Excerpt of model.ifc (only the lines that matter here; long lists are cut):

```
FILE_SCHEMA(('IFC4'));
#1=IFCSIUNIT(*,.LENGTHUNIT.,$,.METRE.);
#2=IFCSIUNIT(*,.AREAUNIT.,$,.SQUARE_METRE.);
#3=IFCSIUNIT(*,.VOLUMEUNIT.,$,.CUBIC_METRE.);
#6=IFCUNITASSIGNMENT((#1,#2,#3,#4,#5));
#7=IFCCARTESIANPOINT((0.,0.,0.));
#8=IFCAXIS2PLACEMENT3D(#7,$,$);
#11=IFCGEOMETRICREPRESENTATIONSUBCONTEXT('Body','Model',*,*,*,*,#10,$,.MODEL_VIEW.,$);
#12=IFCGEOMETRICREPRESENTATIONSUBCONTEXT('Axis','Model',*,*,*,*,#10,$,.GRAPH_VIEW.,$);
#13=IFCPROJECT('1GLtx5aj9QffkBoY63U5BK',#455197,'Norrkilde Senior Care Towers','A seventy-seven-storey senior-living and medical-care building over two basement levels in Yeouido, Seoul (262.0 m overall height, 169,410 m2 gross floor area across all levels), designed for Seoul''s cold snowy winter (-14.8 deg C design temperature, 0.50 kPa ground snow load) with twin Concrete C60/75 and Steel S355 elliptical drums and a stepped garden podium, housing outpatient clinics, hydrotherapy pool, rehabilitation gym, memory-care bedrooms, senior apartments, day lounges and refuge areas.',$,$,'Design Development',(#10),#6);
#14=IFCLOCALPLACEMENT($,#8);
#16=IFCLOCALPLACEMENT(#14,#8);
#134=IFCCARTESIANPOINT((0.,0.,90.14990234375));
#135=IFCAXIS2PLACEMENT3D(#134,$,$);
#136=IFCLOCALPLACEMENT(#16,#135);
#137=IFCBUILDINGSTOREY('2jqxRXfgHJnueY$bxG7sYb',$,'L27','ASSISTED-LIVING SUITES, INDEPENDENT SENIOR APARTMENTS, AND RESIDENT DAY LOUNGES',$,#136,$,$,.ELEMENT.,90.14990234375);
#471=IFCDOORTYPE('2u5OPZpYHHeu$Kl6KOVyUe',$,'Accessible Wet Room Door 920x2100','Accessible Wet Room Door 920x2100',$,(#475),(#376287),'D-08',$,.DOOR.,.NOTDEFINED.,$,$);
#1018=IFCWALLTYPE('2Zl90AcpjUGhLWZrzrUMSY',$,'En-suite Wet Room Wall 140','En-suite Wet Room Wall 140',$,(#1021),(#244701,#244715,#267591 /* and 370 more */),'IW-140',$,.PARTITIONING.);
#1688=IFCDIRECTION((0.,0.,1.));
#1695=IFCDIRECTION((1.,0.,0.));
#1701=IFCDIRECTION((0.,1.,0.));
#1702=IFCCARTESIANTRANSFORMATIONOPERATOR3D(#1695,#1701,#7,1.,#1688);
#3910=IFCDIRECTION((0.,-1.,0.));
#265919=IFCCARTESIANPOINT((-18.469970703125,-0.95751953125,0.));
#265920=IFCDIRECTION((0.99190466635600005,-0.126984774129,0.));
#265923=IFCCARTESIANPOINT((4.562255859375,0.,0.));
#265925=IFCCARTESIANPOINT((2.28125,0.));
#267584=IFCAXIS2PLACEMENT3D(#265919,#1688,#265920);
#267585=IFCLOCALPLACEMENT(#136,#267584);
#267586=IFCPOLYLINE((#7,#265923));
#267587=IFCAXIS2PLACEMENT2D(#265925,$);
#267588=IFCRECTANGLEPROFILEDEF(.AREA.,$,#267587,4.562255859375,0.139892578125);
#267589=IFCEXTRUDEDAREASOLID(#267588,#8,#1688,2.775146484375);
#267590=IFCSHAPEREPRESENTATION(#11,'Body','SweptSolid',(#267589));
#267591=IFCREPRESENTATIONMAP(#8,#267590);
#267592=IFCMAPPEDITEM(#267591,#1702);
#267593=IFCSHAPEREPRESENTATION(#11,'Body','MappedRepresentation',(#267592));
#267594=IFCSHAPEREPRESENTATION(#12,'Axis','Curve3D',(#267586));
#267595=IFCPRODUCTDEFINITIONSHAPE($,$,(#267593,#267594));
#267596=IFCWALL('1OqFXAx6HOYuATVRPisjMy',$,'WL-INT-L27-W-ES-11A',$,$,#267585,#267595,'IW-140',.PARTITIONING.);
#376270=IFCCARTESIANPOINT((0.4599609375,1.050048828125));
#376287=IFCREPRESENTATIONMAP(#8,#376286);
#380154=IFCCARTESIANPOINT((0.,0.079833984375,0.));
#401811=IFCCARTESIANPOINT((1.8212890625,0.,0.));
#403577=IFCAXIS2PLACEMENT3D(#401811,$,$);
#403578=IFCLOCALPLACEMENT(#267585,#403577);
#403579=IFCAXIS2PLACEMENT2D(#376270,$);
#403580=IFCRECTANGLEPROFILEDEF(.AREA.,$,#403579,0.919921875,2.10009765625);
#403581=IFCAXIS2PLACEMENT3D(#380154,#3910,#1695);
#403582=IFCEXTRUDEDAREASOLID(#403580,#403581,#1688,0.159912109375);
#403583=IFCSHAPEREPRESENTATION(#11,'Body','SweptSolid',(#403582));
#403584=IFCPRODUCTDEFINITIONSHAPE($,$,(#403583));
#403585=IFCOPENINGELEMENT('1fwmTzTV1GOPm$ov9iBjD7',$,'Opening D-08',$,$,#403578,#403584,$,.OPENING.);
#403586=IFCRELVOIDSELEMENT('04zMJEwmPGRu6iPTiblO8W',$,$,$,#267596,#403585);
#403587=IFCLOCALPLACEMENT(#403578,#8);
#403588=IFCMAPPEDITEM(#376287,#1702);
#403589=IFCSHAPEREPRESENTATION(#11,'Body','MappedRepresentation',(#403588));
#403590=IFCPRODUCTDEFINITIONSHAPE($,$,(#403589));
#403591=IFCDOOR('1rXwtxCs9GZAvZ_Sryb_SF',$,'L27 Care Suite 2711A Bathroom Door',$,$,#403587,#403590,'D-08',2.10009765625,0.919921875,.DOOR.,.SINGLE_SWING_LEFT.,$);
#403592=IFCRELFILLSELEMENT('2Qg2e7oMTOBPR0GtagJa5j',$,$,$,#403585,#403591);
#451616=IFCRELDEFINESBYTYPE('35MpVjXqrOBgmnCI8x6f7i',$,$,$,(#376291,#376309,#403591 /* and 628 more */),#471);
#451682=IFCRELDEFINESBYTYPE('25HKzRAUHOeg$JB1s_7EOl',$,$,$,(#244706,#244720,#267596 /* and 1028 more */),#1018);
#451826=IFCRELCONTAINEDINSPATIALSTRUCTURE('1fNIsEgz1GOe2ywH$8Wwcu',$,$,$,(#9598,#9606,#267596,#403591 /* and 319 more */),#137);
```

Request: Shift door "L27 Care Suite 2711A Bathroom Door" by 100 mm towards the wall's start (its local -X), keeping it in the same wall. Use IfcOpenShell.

```python
import ifcopenshell
import ifcopenshell.api.geometry
import ifcopenshell.util.placement
import ifcopenshell.util.unit

model = ifcopenshell.open("model.ifc")
unit_scale = ifcopenshell.util.unit.calculate_unit_scale(model)

door = model.by_guid("1rXwtxCs9GZAvZ_Sryb_SF")
opening = door.FillsVoids[0].RelatingOpeningElement
wall = opening.VoidsElements[0].RelatingBuildingElement

wall_matrix = ifcopenshell.util.placement.get_local_placement(wall.ObjectPlacement)
shift = wall_matrix[:3, 0] * -0.1 / unit_scale
before = ifcopenshell.util.placement.get_local_placement(door.ObjectPlacement)[:3, 3].copy()

# The door is placed relative to its opening, so it follows when the opening moves.
matrix = ifcopenshell.util.placement.get_local_placement(opening.ObjectPlacement)
matrix[:3, 3] += shift
ifcopenshell.api.geometry.edit_object_placement(
    model, product=opening, matrix=matrix, is_si=False, should_transform_children=True
)

after = ifcopenshell.util.placement.get_local_placement(door.ObjectPlacement)[:3, 3]
print("door moved by", (after - before).round(3) + 0.0)

model.write("model_updated.ifc")
```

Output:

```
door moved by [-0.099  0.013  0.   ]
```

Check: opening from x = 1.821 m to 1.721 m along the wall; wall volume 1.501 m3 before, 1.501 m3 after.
